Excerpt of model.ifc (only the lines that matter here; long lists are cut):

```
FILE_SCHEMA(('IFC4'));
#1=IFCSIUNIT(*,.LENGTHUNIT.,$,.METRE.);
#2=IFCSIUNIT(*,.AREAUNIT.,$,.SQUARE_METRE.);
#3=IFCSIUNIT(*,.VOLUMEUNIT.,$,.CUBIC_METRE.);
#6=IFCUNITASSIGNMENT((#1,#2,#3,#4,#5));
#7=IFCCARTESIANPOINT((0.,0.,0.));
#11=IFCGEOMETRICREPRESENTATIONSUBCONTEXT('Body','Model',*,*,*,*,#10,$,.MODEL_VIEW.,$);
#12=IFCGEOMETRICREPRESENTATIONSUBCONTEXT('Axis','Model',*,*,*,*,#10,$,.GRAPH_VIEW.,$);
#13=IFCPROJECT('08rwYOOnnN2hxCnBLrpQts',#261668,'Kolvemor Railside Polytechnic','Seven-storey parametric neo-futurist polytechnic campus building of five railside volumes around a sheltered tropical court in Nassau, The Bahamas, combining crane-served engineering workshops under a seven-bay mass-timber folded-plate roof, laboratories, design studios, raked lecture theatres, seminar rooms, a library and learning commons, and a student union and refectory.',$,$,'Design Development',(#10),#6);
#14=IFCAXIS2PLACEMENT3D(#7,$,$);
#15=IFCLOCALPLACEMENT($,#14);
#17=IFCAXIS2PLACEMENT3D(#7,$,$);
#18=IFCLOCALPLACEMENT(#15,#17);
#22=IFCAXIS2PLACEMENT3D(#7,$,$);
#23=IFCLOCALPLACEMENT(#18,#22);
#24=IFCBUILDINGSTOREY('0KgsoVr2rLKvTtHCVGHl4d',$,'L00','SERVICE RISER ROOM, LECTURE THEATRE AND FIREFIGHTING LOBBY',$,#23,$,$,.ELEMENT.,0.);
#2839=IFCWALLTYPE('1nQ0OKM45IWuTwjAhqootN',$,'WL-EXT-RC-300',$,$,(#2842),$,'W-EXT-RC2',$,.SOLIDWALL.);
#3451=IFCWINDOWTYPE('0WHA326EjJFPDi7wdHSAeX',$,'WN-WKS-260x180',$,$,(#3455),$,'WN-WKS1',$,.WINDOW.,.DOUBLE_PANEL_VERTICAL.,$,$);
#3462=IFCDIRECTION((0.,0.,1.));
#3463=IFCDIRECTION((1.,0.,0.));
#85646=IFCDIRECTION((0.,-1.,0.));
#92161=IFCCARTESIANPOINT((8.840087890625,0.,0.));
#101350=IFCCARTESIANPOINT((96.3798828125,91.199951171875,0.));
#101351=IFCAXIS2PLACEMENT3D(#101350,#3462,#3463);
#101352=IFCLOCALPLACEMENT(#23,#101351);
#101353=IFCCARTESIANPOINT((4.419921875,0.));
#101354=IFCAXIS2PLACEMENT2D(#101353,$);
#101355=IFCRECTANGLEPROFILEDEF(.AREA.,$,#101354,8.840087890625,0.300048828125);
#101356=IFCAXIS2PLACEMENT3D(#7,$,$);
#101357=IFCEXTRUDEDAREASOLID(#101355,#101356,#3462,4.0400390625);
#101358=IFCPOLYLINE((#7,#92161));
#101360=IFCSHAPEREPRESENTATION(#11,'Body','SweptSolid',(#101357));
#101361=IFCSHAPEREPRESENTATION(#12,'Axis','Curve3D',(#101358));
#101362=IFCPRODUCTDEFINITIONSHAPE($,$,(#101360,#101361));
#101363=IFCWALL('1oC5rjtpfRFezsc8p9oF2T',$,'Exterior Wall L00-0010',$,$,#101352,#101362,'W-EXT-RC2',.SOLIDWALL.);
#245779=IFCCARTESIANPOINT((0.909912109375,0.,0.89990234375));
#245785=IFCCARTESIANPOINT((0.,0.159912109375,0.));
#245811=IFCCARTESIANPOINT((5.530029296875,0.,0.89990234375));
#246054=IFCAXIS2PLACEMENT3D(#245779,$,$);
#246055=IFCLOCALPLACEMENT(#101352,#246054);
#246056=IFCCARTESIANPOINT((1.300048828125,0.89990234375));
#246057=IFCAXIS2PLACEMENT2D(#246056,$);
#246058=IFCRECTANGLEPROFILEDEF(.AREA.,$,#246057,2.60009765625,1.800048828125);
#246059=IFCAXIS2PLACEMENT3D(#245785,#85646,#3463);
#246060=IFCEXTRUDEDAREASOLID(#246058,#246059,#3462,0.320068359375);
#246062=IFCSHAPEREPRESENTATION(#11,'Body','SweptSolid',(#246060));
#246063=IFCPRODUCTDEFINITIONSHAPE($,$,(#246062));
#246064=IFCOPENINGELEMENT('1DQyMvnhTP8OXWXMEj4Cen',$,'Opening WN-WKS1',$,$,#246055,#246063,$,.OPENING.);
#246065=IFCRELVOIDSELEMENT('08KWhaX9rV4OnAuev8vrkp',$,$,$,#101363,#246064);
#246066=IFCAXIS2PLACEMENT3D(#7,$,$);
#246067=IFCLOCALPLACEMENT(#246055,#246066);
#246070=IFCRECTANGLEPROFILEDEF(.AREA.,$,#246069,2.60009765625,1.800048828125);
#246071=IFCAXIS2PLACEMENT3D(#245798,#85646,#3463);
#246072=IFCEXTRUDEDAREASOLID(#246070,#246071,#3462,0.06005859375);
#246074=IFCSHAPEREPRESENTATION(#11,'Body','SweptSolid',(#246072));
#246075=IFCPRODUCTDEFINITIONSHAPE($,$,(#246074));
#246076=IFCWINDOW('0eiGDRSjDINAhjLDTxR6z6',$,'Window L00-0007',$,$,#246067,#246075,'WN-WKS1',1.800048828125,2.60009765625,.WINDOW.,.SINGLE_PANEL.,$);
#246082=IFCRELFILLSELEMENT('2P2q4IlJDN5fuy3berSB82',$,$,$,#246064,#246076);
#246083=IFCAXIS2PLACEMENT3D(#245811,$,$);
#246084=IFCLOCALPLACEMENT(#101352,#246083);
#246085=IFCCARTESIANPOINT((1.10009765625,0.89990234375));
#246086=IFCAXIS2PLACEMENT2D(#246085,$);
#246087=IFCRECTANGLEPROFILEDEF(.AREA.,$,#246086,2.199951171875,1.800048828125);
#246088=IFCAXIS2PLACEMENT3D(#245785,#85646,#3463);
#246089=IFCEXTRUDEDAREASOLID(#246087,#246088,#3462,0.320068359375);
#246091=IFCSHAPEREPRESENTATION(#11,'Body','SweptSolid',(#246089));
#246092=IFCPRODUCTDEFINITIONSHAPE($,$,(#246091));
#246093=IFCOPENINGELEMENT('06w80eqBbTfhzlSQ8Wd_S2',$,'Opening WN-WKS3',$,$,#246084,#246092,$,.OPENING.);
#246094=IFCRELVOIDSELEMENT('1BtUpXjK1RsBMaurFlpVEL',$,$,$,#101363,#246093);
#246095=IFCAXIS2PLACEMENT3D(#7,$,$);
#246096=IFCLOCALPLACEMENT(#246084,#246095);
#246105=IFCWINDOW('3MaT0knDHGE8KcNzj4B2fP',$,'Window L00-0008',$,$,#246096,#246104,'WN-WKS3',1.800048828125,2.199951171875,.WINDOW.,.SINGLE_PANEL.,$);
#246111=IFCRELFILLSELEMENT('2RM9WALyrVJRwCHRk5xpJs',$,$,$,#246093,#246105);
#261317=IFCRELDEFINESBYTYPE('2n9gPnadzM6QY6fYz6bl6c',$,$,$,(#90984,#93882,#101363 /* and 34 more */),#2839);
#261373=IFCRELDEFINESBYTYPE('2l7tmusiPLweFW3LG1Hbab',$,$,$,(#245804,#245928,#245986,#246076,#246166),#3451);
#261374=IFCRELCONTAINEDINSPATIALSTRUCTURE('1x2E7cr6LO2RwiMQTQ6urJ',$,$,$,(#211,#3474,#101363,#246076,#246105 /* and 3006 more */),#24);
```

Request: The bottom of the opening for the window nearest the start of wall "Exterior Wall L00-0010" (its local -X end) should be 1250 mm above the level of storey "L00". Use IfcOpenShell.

```python
import numpy as np
import ifcopenshell
import ifcopenshell.api.geometry
import ifcopenshell.geom
import ifcopenshell.util.element
import ifcopenshell.util.placement
import ifcopenshell.util.shape
import ifcopenshell.util.unit

model = ifcopenshell.open("model.ifc")
unit_scale = ifcopenshell.util.unit.calculate_unit_scale(model)

window = model.by_guid("0eiGDRSjDINAhjLDTxR6z6")
opening = window.FillsVoids[0].RelatingOpeningElement
storey = ifcopenshell.util.element.get_container(window, ifc_class="IfcBuildingStorey")
level = ifcopenshell.util.placement.get_local_placement(storey.ObjectPlacement)[2, 3]

# The opening's origin need not be at the sill, so measure its lowest point.
shape = ifcopenshell.geom.create_shape(ifcopenshell.geom.settings(), opening)
bottom = ifcopenshell.util.shape.get_shape_bottom_elevation(shape, shape.geometry) / unit_scale
dz = level + 1.25 / unit_scale - bottom

shift = np.array([0.0, 0.0, dz])
# The window is placed relative to its opening, so it follows when the opening moves.
matrix = ifcopenshell.util.placement.get_local_placement(opening.ObjectPlacement)
matrix[:3, 3] += shift
ifcopenshell.api.geometry.edit_object_placement(
    model, product=opening, matrix=matrix, is_si=False, should_transform_children=True
)

print(f"moved by {dz * unit_scale:+.3f} m")

model.write("model-out.ifc")
```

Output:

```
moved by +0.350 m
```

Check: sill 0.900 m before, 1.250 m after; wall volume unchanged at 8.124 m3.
